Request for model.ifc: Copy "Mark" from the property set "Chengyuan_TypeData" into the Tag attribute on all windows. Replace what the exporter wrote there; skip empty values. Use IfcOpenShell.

First a look at what the model holds.

```python
import ifcopenshell
import ifcopenshell.util.element

model = ifcopenshell.open("model.ifc")
print(model.schema)
windows = model.by_type("IfcWindow")
print(len(windows), "windows")
for e in windows[:8]:
    source = ifcopenshell.util.element.get_pset(e, "Chengyuan_TypeData", "Mark")
    target = e.Tag
    print(e.id(), repr(source), repr(target), sep=" | ")
```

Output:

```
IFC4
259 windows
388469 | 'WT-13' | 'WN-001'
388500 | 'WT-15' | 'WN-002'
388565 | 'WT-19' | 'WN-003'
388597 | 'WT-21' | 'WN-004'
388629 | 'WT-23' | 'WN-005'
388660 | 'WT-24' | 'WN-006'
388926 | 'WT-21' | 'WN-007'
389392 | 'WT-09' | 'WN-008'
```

```python
import ifcopenshell
import ifcopenshell.util.element

model = ifcopenshell.open("model.ifc")

count = 0
for e in model.by_type("IfcWindow"):
    value = ifcopenshell.util.element.get_pset(e, "Chengyuan_TypeData", "Mark")
    current = e.Tag
    if not value or not value.strip() or current == value:
        continue
    e.Tag = value
    count += 1

print(count, "windows updated")

model.write("model_updated.ifc")
```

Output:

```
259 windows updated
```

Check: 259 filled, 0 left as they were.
